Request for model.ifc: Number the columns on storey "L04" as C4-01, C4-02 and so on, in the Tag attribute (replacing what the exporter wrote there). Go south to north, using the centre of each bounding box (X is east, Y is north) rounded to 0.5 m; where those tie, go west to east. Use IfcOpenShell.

First a look at what the model holds.

```python
import ifcopenshell
import ifcopenshell.util.element
import ifcopenshell.util.placement

model = ifcopenshell.open("model.ifc")
print(model.schema)
storey = next(s for s in model.by_type("IfcBuildingStorey") if s.Name == "L04")
columns = [e for e in ifcopenshell.util.element.get_decomposition(storey) if e.is_a("IfcColumn")]
for e in sorted(columns, key=lambda e: e.id()):
    origin = ifcopenshell.util.placement.get_local_placement(e.ObjectPlacement)[:3, 3]
    print(e.id(), e.Tag, e.Name, origin.round(2) + 0.0, sep=" | ")
```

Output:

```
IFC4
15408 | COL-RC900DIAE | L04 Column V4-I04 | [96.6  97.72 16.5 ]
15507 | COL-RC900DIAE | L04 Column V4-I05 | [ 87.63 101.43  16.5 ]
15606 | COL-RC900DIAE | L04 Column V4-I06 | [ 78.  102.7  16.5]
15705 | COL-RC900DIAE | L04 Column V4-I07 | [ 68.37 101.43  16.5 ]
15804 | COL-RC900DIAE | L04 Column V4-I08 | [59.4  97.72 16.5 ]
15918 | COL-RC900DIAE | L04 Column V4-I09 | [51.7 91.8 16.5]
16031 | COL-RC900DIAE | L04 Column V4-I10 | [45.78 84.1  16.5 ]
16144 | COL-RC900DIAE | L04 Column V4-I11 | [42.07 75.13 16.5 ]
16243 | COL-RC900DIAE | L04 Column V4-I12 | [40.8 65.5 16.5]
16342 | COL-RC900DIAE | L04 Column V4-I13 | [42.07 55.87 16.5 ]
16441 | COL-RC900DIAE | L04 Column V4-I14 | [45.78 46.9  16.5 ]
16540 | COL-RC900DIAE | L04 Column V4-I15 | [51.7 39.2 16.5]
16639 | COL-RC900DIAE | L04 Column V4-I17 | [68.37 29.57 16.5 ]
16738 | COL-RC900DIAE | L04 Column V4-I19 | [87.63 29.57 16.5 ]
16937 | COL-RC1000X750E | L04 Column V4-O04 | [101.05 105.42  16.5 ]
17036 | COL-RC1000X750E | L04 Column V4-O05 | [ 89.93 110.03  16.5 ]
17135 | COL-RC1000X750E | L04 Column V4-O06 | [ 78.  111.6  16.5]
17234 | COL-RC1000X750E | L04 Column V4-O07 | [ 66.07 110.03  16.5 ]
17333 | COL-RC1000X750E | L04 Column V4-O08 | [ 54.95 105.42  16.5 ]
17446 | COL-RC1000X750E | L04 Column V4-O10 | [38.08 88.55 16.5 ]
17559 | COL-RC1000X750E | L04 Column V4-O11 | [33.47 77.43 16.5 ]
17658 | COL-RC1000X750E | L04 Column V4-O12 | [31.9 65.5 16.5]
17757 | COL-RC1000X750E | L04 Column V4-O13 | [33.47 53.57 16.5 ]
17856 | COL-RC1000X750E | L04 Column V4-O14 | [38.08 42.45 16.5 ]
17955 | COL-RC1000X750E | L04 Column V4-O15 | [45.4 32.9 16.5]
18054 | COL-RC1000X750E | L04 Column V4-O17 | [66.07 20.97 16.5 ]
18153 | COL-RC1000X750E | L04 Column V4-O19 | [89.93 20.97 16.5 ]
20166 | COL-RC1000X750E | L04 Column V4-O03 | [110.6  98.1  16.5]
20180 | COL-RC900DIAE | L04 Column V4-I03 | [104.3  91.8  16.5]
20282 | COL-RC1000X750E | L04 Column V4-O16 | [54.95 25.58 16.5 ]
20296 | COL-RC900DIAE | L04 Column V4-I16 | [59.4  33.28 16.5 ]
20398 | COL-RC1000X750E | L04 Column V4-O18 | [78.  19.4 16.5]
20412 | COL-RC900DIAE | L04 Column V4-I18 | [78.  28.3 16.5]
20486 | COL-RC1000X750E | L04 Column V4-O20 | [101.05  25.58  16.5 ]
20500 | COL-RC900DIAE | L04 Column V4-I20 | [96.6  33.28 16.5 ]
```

```python
import ifcopenshell
import ifcopenshell.geom
import ifcopenshell.util.element
import ifcopenshell.util.shape

model = ifcopenshell.open("model.ifc")
settings = ifcopenshell.geom.settings()
settings.set("use-world-coords", True)


def centre(element):
    shape = ifcopenshell.geom.create_shape(settings, element)
    return ifcopenshell.util.shape.get_bbox_centroid(shape.geometry)


storey = next(s for s in model.by_type("IfcBuildingStorey") if s.Name == "L04")
columns = [e for e in ifcopenshell.util.element.get_decomposition(storey) if e.is_a("IfcColumn")]

# Insertion points can sit at a corner or the storey origin, so sort by the geometry (in metres).
centres = {e: centre(e) for e in columns}
columns.sort(key=lambda e: (round(centres[e][1] / 0.5), centres[e][0]))

for i, e in enumerate(columns, start=1):
    number = f"C4-{i:02d}"
    e.Tag = number
    print(e.id(), number)

model.write("model_v2.ifc")
```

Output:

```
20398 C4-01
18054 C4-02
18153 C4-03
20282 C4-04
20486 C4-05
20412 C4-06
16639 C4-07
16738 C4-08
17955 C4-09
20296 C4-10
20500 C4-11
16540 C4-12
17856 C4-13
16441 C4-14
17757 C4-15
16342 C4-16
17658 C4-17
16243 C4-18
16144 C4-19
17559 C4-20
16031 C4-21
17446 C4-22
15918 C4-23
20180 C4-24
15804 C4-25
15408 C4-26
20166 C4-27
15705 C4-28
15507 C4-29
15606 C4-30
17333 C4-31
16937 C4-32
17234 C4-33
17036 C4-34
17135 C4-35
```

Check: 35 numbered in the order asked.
